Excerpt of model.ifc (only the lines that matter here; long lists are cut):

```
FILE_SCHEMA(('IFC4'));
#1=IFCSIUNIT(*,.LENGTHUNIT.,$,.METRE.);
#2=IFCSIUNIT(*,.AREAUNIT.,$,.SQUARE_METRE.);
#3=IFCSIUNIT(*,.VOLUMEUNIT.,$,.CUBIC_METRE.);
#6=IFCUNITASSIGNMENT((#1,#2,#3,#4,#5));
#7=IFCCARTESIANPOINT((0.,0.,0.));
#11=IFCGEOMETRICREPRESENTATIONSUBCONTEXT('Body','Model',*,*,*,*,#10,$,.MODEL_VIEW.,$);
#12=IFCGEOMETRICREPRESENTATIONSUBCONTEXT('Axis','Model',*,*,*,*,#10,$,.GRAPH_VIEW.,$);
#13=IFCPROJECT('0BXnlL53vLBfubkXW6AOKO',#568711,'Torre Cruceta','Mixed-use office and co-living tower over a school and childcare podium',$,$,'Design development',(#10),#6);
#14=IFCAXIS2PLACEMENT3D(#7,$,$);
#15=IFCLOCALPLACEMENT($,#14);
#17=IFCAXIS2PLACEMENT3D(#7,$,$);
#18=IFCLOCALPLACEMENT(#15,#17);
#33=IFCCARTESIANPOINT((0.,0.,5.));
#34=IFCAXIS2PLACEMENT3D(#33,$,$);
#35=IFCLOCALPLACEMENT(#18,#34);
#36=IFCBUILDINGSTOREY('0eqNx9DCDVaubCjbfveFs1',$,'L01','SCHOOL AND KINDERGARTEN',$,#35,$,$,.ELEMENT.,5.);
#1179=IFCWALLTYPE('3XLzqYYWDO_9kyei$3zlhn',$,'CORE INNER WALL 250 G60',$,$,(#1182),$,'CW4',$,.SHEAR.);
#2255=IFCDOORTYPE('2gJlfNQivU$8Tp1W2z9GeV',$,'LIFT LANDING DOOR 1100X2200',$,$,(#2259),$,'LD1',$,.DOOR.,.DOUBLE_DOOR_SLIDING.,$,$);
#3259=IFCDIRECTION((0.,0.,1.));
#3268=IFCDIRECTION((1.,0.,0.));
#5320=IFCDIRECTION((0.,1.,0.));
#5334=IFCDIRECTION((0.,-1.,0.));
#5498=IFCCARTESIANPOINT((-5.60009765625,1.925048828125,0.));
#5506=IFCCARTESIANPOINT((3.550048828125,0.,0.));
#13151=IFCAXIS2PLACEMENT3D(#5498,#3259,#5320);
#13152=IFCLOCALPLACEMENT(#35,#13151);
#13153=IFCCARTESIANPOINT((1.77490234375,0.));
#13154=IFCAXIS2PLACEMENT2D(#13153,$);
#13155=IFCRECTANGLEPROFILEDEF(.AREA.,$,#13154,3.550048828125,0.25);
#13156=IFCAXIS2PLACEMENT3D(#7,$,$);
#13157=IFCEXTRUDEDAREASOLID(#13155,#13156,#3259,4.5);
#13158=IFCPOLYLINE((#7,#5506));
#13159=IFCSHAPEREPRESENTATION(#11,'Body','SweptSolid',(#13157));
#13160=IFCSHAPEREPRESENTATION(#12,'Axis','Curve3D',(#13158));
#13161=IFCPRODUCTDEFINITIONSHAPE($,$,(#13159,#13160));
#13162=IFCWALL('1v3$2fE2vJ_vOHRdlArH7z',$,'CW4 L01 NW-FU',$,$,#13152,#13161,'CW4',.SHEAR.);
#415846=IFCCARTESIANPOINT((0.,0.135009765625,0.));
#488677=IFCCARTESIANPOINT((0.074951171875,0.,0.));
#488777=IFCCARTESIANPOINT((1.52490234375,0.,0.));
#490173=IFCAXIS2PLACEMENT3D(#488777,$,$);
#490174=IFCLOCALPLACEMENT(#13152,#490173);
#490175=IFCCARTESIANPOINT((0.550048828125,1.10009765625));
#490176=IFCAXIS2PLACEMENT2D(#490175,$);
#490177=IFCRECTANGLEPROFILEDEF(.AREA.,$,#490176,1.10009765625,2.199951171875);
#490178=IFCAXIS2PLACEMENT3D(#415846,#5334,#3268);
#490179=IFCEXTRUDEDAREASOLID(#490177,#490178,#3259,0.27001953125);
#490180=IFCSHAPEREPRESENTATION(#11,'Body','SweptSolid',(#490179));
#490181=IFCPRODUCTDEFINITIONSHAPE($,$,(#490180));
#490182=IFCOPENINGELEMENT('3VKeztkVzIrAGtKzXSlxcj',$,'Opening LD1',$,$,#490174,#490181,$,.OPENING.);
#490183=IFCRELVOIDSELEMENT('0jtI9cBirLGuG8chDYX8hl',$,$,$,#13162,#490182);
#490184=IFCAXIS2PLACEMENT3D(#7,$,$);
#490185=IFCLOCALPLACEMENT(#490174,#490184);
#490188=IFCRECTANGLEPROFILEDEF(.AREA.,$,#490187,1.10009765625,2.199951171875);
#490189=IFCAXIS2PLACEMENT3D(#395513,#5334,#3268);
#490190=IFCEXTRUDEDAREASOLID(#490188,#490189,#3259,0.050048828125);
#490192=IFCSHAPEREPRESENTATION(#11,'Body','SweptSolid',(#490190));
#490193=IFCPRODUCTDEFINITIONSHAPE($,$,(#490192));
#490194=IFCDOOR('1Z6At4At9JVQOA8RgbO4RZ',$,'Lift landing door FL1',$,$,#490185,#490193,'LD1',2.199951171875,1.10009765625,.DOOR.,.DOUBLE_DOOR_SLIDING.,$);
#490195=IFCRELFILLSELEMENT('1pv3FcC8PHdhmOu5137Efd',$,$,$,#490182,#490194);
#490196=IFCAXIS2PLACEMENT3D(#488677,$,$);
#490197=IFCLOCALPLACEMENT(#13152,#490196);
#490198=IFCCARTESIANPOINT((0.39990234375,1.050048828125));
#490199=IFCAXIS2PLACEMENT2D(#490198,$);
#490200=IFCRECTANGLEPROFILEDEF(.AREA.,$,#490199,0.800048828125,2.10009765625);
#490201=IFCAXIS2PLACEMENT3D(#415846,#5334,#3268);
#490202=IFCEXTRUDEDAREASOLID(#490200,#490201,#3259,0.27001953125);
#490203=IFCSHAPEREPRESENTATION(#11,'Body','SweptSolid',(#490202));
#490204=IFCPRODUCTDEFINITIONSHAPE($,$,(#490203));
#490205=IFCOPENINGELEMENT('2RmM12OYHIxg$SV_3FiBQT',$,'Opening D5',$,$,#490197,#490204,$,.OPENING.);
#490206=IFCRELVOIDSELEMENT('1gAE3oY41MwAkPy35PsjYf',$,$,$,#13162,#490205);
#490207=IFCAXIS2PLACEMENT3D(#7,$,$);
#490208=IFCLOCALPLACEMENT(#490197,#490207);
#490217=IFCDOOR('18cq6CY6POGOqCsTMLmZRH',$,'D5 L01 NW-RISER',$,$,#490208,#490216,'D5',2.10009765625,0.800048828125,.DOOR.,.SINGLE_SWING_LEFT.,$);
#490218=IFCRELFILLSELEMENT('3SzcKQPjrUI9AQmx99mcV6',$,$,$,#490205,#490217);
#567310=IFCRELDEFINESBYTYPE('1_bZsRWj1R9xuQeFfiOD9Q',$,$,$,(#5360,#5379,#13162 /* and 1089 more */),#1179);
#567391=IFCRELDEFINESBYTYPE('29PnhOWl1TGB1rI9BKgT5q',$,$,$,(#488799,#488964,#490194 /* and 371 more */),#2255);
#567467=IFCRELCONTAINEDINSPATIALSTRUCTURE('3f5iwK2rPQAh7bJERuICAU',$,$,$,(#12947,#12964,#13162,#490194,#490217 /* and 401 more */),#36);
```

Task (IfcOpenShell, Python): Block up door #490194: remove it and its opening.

```python
import ifcopenshell
import ifcopenshell.api.feature
import ifcopenshell.api.root
import ifcopenshell.geom
import ifcopenshell.util.shape

model = ifcopenshell.open("model.ifc")
settings = ifcopenshell.geom.settings()


def volume(element):
    """Net volume in cubic metres, openings subtracted."""
    shape = ifcopenshell.geom.create_shape(settings, element)
    return ifcopenshell.util.shape.get_volume(shape.geometry)


door = model.by_id(490194)
opening = door.FillsVoids[0].RelatingOpeningElement
wall = opening.VoidsElements[0].RelatingBuildingElement
before = volume(wall)

ifcopenshell.api.root.remove_product(model, product=door)
ifcopenshell.api.feature.remove_feature(model, feature=opening)

after = volume(wall)

print(f"wall volume {before:.3f} -> {after:.3f} m3")

model.write("model_updated.ifc")
```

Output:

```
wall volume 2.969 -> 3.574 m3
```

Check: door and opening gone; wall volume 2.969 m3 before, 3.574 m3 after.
